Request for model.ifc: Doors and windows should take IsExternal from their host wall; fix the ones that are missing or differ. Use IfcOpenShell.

First a look at what the model holds.

```python
import ifcopenshell
import ifcopenshell.util.element

model = ifcopenshell.open("model.ifc")
print(model.schema)
seen = {}
for e in model.by_type("IfcDoor") + model.by_type("IfcWindow"):
    if not e.FillsVoids:
        continue
    host = e.FillsVoids[0].RelatingOpeningElement.VoidsElements[0].RelatingBuildingElement
    own = ifcopenshell.util.element.get_pset(e, f"Pset_{e.is_a()[3:].removesuffix('StandardCase')}Common", "IsExternal")
    wall = ifcopenshell.util.element.get_pset(host, "Pset_WallCommon", "IsExternal")
    seen[e.is_a(), own, wall] = seen.get((e.is_a(), own, wall), 0) + 1
for (cls, own, wall), count in sorted(seen.items(), key=str):
    print(count, cls, "IsExternal:", own, "| host wall:", wall)
```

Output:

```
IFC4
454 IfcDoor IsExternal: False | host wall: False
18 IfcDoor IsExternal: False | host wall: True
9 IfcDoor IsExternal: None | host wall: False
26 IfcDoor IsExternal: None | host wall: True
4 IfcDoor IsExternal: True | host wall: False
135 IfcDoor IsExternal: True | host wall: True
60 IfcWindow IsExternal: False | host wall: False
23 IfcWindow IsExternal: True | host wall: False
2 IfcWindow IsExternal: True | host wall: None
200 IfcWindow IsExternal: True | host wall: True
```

```python
import ifcopenshell
import ifcopenshell.api.pset
import ifcopenshell.util.element

model = ifcopenshell.open("model.ifc")

count = 0
for ifc_class, pset_name in (("IfcDoor", "Pset_DoorCommon"), ("IfcWindow", "Pset_WindowCommon")):
    for e in model.by_type(ifc_class):
        if not e.FillsVoids:
            continue
        host = e.FillsVoids[0].RelatingOpeningElement.VoidsElements[0].RelatingBuildingElement
        external = ifcopenshell.util.element.get_pset(host, "Pset_WallCommon", "IsExternal")
        if external is None or ifcopenshell.util.element.get_pset(e, pset_name, "IsExternal") == external:
            continue
        pset = ifcopenshell.api.pset.add_pset(model, product=e, name=pset_name)
        ifcopenshell.api.pset.edit_pset(model, pset=pset, properties={"IsExternal": external})
        count += 1

print(count, "updated")

model.write("model_edited.ifc")
```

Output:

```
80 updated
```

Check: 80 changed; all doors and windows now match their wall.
